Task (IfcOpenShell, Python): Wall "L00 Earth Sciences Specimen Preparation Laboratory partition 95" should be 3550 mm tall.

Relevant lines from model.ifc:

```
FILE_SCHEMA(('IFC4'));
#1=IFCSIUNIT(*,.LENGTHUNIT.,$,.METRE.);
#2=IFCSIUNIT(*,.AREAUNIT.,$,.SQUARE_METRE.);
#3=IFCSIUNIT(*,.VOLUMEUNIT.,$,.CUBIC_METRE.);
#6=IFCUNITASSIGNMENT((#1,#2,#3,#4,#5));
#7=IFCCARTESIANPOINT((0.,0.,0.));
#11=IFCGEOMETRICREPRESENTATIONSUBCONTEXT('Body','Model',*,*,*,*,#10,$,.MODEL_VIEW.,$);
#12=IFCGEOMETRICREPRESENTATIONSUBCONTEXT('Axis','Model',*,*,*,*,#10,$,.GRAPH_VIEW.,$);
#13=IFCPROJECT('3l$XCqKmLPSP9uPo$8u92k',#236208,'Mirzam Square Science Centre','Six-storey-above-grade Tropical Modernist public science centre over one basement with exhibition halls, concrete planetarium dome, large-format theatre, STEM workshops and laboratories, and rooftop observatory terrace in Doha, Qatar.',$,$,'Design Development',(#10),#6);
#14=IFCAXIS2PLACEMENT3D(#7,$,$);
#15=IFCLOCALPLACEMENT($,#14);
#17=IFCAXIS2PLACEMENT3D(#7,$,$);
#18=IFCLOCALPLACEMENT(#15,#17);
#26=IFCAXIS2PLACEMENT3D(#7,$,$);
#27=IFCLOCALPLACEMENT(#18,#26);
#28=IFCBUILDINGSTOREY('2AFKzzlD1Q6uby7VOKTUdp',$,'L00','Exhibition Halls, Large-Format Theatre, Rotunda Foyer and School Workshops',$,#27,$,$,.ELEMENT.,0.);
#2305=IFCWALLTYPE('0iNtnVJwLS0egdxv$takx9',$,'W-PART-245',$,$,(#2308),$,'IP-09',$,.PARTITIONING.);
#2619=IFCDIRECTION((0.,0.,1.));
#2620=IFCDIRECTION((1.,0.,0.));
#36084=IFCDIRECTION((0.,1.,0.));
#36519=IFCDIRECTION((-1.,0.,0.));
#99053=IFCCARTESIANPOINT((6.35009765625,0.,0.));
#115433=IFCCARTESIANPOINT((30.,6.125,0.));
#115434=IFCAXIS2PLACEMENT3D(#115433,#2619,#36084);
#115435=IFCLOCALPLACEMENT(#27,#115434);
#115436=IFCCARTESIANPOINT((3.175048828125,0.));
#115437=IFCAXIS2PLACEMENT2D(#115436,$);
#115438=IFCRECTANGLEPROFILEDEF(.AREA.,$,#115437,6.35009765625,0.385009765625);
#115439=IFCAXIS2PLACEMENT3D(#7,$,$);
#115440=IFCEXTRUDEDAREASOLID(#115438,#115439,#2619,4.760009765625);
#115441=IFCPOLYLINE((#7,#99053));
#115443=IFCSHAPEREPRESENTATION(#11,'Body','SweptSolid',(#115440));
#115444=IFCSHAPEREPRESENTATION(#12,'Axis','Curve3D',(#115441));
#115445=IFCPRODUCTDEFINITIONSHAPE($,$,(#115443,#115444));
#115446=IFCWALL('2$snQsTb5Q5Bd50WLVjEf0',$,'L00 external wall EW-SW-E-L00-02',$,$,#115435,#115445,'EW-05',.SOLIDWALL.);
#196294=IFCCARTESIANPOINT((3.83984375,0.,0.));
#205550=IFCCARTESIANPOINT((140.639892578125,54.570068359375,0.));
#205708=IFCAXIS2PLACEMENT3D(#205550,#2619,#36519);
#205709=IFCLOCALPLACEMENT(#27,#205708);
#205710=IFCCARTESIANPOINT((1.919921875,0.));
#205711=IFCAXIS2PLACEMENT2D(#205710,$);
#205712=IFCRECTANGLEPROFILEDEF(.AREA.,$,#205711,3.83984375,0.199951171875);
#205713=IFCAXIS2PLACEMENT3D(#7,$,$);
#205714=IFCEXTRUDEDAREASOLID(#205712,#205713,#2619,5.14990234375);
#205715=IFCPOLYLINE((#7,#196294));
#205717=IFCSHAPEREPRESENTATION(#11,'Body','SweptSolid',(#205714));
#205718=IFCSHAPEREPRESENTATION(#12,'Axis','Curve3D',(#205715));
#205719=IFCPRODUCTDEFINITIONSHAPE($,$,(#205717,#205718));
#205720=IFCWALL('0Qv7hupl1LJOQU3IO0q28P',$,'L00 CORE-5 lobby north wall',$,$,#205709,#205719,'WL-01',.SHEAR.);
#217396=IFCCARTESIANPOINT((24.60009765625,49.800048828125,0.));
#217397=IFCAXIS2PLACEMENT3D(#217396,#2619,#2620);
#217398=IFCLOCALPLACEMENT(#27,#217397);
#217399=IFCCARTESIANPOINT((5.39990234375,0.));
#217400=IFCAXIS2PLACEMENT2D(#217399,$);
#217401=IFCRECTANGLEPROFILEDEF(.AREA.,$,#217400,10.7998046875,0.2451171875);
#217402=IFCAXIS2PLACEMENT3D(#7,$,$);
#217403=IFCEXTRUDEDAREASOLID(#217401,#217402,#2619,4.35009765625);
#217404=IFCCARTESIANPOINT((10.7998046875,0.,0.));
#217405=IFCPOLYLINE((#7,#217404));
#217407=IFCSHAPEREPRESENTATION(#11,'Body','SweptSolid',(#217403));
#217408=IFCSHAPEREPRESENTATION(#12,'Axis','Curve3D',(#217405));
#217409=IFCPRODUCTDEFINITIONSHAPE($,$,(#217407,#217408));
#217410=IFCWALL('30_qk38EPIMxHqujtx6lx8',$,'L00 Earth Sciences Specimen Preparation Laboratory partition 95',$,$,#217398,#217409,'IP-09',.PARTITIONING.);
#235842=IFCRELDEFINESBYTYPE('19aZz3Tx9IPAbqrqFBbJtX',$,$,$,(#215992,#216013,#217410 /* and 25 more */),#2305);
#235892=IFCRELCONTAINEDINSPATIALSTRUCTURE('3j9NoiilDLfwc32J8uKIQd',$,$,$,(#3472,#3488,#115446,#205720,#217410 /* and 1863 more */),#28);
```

```python
import ifcopenshell
import ifcopenshell.geom
import ifcopenshell.util.representation
import ifcopenshell.util.shape
import ifcopenshell.util.unit

model = ifcopenshell.open("model.ifc")
unit_scale = ifcopenshell.util.unit.calculate_unit_scale(model)
settings = ifcopenshell.geom.settings()


def volume(element):
    """Net volume in cubic metres, openings subtracted."""
    shape = ifcopenshell.geom.create_shape(settings, element)
    return ifcopenshell.util.shape.get_volume(shape.geometry)


wall = model.by_id(217410)
before = volume(wall)

body = ifcopenshell.util.representation.get_representation(wall, "Model", "Body")
solid = body.Items[0]
old_height = solid.Depth
solid.Depth = 3.55 / unit_scale
after = volume(wall)

print(f"height {old_height:g} -> {solid.Depth:g}, volume {before:.3f} -> {after:.3f} m3")

model.write("model_updated.ifc")
```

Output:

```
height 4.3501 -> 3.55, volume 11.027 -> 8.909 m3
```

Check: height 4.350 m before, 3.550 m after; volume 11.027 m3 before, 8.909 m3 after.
